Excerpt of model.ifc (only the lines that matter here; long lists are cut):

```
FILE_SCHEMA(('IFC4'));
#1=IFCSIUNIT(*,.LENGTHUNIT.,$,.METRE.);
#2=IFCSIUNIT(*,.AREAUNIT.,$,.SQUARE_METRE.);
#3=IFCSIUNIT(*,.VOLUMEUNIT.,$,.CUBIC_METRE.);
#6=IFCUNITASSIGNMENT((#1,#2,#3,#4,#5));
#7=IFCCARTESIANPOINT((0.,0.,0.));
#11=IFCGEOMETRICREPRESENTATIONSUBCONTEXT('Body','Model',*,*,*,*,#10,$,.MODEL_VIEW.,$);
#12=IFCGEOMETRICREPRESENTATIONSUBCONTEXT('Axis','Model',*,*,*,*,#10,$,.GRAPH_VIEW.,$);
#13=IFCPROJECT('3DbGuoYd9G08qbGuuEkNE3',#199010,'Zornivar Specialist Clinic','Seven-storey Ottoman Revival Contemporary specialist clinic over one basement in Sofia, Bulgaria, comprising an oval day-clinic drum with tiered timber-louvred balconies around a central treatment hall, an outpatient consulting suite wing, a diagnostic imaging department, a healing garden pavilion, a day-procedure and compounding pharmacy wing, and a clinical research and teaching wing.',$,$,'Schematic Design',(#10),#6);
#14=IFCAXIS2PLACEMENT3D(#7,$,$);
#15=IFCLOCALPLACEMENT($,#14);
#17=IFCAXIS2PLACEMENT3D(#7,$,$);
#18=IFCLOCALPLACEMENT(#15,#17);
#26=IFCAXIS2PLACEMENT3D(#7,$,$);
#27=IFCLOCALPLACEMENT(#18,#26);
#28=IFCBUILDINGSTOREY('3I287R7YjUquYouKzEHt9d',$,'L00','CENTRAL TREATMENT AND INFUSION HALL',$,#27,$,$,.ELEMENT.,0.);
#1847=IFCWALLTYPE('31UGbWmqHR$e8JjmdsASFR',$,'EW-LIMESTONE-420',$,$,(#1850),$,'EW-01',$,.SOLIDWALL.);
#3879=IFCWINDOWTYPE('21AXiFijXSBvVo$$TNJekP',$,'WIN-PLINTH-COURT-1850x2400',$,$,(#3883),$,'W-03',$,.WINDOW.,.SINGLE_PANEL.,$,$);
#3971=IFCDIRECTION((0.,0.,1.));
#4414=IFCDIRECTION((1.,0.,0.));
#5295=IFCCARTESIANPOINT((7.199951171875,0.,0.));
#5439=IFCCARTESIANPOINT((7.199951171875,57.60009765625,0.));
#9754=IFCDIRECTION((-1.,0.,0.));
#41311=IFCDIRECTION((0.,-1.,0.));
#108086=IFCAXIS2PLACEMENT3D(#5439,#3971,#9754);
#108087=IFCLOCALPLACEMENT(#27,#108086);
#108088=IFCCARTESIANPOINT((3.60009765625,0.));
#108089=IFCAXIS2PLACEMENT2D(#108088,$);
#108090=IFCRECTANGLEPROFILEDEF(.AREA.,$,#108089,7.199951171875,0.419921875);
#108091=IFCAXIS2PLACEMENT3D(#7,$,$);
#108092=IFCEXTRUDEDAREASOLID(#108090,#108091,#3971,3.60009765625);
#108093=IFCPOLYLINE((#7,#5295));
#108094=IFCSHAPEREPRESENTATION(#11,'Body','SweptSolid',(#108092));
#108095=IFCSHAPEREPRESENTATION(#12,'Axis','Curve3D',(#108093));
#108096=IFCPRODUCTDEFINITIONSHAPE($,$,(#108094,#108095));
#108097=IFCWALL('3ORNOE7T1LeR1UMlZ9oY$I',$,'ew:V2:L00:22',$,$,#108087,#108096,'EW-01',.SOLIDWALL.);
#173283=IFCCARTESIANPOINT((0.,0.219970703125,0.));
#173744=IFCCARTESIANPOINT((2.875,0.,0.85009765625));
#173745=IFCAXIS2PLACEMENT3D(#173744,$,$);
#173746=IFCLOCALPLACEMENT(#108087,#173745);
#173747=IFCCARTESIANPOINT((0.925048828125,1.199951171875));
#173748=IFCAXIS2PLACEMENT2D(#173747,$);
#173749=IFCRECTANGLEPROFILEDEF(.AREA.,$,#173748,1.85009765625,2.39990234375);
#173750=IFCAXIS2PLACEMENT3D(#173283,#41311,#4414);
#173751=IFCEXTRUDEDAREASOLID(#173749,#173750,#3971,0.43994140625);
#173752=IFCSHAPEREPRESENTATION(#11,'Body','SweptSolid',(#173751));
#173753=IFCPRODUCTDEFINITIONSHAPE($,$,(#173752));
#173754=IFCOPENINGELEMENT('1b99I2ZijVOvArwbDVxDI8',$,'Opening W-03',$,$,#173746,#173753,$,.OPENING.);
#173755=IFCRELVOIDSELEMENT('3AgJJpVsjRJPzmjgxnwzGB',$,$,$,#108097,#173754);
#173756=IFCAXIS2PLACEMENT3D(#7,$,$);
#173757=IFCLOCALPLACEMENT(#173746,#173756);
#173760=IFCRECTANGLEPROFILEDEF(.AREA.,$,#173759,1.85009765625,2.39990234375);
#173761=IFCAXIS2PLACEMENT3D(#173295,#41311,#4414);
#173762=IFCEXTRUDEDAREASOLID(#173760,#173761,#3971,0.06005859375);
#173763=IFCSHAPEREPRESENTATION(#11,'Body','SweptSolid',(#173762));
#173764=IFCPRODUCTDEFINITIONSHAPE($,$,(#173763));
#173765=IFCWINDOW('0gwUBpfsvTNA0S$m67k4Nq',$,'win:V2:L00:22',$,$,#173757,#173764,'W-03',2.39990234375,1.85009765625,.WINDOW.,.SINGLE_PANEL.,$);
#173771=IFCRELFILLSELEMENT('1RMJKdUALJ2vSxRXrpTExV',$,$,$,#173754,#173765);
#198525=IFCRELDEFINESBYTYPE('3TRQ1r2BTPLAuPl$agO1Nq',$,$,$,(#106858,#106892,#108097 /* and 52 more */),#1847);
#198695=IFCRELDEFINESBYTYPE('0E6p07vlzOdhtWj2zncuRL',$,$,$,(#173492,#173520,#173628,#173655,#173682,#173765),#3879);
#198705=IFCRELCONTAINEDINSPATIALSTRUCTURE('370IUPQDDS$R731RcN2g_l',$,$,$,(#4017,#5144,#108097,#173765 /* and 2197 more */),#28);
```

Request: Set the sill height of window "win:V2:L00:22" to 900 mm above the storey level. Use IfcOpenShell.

```python
import numpy as np
import ifcopenshell
import ifcopenshell.api.geometry
import ifcopenshell.geom
import ifcopenshell.util.element
import ifcopenshell.util.placement
import ifcopenshell.util.shape
import ifcopenshell.util.unit

model = ifcopenshell.open("model.ifc")
unit_scale = ifcopenshell.util.unit.calculate_unit_scale(model)

window = model.by_guid("0gwUBpfsvTNA0S$m67k4Nq")
opening = window.FillsVoids[0].RelatingOpeningElement
storey = ifcopenshell.util.element.get_container(window, ifc_class="IfcBuildingStorey")
level = ifcopenshell.util.placement.get_local_placement(storey.ObjectPlacement)[2, 3]

# The opening's origin need not be at the sill, so measure its lowest point.
shape = ifcopenshell.geom.create_shape(ifcopenshell.geom.settings(), opening)
bottom = ifcopenshell.util.shape.get_shape_bottom_elevation(shape, shape.geometry) / unit_scale
dz = level + 0.9 / unit_scale - bottom

shift = np.array([0.0, 0.0, dz])
# The window is placed relative to its opening, so it follows when the opening moves.
matrix = ifcopenshell.util.placement.get_local_placement(opening.ObjectPlacement)
matrix[:3, 3] += shift
ifcopenshell.api.geometry.edit_object_placement(
    model, product=opening, matrix=matrix, is_si=False, should_transform_children=True
)

print(f"moved by {dz * unit_scale:+.3f} m")

model.write("model-out.ifc")
```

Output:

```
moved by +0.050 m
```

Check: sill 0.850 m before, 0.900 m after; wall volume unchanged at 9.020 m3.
